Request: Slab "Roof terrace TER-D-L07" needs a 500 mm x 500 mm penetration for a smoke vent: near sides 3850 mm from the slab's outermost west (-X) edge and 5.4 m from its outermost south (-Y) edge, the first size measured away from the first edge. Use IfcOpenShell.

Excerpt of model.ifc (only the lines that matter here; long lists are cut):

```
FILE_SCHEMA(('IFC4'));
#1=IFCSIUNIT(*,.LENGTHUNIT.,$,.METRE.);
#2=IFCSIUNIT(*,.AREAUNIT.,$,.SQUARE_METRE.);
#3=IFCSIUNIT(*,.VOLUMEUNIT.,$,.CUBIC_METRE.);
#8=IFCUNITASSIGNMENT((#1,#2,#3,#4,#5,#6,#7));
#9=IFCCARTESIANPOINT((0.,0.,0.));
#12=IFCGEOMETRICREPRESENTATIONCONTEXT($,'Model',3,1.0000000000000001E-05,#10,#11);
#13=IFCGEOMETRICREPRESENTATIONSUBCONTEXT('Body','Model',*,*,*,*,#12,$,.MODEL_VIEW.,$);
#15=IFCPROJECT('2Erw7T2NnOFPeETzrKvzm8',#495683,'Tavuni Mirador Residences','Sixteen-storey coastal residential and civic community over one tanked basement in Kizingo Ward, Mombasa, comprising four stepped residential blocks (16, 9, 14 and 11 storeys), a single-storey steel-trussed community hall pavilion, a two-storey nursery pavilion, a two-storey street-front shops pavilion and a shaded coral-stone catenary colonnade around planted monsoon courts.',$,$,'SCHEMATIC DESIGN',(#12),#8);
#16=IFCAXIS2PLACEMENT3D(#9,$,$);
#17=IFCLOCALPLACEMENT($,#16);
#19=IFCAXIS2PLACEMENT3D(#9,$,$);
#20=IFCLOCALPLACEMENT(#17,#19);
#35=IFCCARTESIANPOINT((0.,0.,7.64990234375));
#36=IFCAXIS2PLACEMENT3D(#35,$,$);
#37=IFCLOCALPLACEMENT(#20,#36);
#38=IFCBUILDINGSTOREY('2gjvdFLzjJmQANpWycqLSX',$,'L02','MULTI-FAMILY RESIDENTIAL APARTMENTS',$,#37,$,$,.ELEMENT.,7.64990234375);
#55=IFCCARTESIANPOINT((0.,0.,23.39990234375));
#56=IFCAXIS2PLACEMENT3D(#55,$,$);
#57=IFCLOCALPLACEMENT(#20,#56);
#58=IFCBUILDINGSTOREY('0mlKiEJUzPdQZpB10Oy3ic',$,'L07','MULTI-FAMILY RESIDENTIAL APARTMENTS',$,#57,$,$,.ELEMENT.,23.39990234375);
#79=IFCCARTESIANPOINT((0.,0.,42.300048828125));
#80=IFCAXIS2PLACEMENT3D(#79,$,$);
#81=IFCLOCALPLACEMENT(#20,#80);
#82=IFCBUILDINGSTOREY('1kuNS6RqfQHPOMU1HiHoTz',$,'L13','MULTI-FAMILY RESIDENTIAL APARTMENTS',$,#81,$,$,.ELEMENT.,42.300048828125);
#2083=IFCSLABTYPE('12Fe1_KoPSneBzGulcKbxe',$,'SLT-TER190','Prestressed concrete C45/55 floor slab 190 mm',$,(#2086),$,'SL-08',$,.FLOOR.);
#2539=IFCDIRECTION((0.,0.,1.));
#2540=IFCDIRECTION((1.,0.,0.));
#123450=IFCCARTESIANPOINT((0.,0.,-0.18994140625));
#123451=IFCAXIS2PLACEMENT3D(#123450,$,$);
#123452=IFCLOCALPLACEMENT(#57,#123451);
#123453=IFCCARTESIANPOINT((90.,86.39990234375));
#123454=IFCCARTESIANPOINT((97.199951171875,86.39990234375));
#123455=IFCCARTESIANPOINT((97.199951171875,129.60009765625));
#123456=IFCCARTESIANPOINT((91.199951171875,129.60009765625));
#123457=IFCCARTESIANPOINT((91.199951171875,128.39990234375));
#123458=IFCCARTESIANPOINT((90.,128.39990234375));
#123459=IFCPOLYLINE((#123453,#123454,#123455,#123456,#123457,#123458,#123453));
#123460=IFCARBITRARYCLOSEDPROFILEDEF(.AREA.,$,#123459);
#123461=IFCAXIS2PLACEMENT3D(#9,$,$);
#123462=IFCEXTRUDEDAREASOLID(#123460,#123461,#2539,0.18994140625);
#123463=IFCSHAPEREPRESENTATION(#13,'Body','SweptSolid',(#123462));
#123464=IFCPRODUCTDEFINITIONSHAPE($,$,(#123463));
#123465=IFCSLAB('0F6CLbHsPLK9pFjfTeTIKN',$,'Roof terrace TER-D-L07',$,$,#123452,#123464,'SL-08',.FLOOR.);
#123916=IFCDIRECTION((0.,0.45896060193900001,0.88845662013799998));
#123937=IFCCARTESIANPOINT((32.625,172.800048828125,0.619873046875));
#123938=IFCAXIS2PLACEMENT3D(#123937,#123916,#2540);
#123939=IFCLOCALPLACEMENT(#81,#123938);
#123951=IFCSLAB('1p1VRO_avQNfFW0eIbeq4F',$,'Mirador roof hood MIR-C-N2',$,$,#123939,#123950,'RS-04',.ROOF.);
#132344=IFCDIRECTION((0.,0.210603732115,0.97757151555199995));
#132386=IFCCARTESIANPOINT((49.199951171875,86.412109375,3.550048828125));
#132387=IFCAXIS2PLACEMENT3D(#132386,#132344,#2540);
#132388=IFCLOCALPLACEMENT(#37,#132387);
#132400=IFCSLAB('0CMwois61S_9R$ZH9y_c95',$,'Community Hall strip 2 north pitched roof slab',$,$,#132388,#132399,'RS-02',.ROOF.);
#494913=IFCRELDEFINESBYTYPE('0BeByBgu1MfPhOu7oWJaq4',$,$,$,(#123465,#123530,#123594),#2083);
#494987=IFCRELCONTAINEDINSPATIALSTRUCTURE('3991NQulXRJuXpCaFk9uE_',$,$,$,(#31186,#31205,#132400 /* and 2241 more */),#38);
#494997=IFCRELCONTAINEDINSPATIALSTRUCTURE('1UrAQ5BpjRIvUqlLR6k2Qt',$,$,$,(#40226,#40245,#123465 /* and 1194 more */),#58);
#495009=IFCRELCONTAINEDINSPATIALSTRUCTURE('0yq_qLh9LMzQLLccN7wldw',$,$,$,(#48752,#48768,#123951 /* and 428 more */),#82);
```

```python
import numpy as np
import ifcopenshell
import ifcopenshell.api.feature
import ifcopenshell.api.geometry
import ifcopenshell.api.root
import ifcopenshell.geom
import ifcopenshell.util.placement
import ifcopenshell.util.representation
import ifcopenshell.util.shape
import ifcopenshell.util.unit

model = ifcopenshell.open("model.ifc")
unit_scale = ifcopenshell.util.unit.calculate_unit_scale(model)
settings = ifcopenshell.geom.settings()


def volume(element):
    """Net volume in cubic metres, openings subtracted."""
    shape = ifcopenshell.geom.create_shape(settings, element)
    return ifcopenshell.util.shape.get_volume(shape.geometry)


slab = model.by_id(123465)
before = volume(slab)

# Extent in the slab's own axes, in metres. The edges named are its -X and -Y sides.
slab_shape = ifcopenshell.geom.create_shape(settings, slab)
vertices = ifcopenshell.util.shape.get_vertices(slab_shape.geometry)
x_min, y_min, bottom = vertices.min(axis=0)
top = vertices[:, 2].max()

opening = ifcopenshell.api.root.create_entity(model, ifc_class="IfcOpeningElement", name="Smoke vent opening", predefined_type="OPENING")
context = ifcopenshell.util.representation.get_context(model, "Model", "Body", "MODEL_VIEW")
width, depth = 0.5, 0.5
outline = [(0.0, 0.0), (width, 0.0), (width, depth), (0.0, depth), (0.0, 0.0)]
# Overshoot both faces by 50 mm so the cut is clean.
shape = ifcopenshell.api.geometry.add_slab_representation(
    model, context=context, depth=top - bottom + 0.1, polyline=outline
)
ifcopenshell.api.geometry.assign_representation(model, product=opening, representation=shape)

matrix = ifcopenshell.util.placement.get_local_placement(slab.ObjectPlacement)
matrix[:, 3] = matrix @ np.append(np.array([x_min + 3.85, y_min + 5.4, bottom - 0.05]) / unit_scale, 1.0)
ifcopenshell.api.geometry.edit_object_placement(model, product=opening, matrix=matrix, is_si=False)
ifcopenshell.api.feature.add_feature(model, feature=opening, element=slab)

after = volume(slab)

print(f"slab volume {before:.3f} -> {after:.3f} m3")

model.write("model-out.ifc")
```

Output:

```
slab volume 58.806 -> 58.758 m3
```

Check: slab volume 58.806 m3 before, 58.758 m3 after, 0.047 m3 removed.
